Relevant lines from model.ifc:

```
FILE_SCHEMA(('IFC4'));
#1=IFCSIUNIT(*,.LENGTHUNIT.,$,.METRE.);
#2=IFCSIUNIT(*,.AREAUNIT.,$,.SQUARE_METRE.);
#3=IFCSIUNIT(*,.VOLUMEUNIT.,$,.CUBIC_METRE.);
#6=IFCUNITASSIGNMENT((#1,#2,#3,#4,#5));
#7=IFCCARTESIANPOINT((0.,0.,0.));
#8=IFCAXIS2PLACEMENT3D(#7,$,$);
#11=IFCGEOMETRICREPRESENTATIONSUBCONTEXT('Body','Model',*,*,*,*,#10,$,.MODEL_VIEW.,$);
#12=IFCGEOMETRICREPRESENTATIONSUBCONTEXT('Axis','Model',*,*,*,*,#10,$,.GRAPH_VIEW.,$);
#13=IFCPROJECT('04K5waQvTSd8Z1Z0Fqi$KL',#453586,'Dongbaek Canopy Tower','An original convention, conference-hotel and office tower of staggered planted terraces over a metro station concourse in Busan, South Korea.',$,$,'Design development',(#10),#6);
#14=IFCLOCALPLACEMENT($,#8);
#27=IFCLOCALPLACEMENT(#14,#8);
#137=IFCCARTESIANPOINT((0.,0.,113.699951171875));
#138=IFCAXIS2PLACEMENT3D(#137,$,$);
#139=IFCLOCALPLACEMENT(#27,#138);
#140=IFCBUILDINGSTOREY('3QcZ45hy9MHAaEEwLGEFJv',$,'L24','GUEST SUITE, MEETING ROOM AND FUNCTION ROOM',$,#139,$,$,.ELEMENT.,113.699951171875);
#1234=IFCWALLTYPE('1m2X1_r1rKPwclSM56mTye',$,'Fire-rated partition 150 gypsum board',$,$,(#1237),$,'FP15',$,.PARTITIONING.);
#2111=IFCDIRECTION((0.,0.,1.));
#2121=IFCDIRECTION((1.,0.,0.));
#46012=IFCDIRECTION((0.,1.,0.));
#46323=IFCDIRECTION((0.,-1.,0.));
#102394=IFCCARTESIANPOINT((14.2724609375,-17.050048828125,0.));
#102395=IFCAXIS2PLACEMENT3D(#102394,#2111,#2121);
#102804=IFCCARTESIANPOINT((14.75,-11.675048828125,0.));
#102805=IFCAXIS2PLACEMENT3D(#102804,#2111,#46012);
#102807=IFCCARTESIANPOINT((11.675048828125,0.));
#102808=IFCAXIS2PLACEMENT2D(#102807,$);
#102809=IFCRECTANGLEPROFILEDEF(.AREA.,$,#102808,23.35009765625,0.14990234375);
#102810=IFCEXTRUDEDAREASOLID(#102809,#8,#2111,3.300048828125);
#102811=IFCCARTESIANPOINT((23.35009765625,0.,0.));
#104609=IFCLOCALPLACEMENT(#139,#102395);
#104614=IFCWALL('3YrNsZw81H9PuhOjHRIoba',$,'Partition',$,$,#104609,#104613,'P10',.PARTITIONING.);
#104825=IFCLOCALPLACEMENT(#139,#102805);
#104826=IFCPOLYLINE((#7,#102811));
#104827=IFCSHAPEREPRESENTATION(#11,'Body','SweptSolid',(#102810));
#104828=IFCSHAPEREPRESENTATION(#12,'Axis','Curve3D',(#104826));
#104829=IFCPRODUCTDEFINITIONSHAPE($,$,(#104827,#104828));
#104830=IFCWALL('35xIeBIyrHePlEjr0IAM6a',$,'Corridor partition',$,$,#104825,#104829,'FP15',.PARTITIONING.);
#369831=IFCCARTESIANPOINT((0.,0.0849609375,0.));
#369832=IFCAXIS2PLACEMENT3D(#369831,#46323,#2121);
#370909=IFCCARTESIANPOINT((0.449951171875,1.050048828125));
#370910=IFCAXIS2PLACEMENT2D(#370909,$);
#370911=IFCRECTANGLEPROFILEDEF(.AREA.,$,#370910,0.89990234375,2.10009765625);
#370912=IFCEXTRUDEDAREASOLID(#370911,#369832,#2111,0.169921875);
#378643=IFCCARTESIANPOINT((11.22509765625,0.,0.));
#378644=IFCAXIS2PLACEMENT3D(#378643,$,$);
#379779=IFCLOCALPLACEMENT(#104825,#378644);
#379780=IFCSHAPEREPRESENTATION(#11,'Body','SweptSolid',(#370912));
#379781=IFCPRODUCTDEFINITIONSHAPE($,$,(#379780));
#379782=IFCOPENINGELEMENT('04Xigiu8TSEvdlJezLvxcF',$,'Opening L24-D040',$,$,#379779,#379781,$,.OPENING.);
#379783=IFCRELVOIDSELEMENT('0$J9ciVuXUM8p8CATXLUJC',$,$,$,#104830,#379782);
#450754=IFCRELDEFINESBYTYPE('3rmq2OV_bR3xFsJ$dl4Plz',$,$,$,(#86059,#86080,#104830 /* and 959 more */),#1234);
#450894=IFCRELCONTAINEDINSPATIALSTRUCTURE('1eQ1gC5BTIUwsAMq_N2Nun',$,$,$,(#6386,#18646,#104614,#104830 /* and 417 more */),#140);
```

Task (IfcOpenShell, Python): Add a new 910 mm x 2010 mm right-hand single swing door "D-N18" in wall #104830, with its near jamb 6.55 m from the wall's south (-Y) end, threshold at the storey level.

```python
import numpy as np
import ifcopenshell
import ifcopenshell.api.feature
import ifcopenshell.api.geometry
import ifcopenshell.api.root
import ifcopenshell.api.spatial
import ifcopenshell.geom
import ifcopenshell.util.element
import ifcopenshell.util.placement
import ifcopenshell.util.representation
import ifcopenshell.util.shape
import ifcopenshell.util.unit

model = ifcopenshell.open("model.ifc")
unit_scale = ifcopenshell.util.unit.calculate_unit_scale(model)
settings = ifcopenshell.geom.settings()


def volume(element):
    """Net volume in cubic metres, openings subtracted."""
    shape = ifcopenshell.geom.create_shape(settings, element)
    return ifcopenshell.util.shape.get_volume(shape.geometry)


wall = model.by_guid("35xIeBIyrHePlEjr0IAM6a")
storey = ifcopenshell.util.element.get_container(wall, ifc_class="IfcBuildingStorey")
context = ifcopenshell.util.representation.get_context(model, "Model", "Body", "MODEL_VIEW")
before = volume(wall)

width, height, from_end, sill = 0.91, 2.01, 6.55, 0.0  # metres

# The wall runs along its own X axis, and the end named is its -X end.
wall_shape = ifcopenshell.geom.create_shape(settings, wall)
x, y, z = ifcopenshell.util.shape.get_vertices(wall_shape.geometry).T
start = x.min() + from_end
face, thickness = float(y.min()), float(y.max() - y.min())
wall_matrix = ifcopenshell.util.placement.get_local_placement(wall.ObjectPlacement)
level = ifcopenshell.util.placement.get_local_placement(storey.ObjectPlacement)[2, 3]


def in_wall(x, y):
    """Placement at x, y metres in the wall's axes, at sill height."""
    matrix = wall_matrix.copy()
    matrix[:, 3] = wall_matrix @ np.array([x / unit_scale, y / unit_scale, 0.0, 1.0])
    matrix[2, 3] = level + sill / unit_scale
    return matrix


# Opening: a box that overshoots both wall faces by 50 mm.
opening = ifcopenshell.api.root.create_entity(model, ifc_class="IfcOpeningElement", predefined_type="OPENING")
box = ifcopenshell.api.geometry.add_wall_representation(
    model, context=context, length=width, height=height, thickness=thickness + 0.1
)
ifcopenshell.api.geometry.assign_representation(model, product=opening, representation=box)
ifcopenshell.api.geometry.edit_object_placement(model, product=opening, matrix=in_wall(start, face - 0.05), is_si=False)
ifcopenshell.api.feature.add_feature(model, feature=opening, element=wall)

door = ifcopenshell.api.root.create_entity(model, ifc_class="IfcDoor", name="D-N18", predefined_type="DOOR")
door.OverallWidth, door.OverallHeight = width / unit_scale, height / unit_scale
door.OperationType = "SINGLE_SWING_RIGHT"
body = ifcopenshell.api.geometry.add_door_representation(
    model,
    context=context,
    overall_width=door.OverallWidth,
    overall_height=door.OverallHeight,
    operation_type="SINGLE_SWING_RIGHT",
    lining_properties={"LiningDepth": thickness / unit_scale, "ThresholdDepth": thickness / unit_scale},
)
ifcopenshell.api.geometry.assign_representation(model, product=door, representation=body)
ifcopenshell.api.spatial.assign_container(model, products=[door], relating_structure=storey)
ifcopenshell.api.feature.add_filling(model, opening=opening, element=door)

# The lining spans the wall, so the door starts at the wall face.
ifcopenshell.api.geometry.edit_object_placement(model, product=door, matrix=in_wall(start, face), is_si=False)

after = volume(wall)

print(f"wall volume {before:.3f} -> {after:.3f} m3")

model.write("model_v2.ifc")
```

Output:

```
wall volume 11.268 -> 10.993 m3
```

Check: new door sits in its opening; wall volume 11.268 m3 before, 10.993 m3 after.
